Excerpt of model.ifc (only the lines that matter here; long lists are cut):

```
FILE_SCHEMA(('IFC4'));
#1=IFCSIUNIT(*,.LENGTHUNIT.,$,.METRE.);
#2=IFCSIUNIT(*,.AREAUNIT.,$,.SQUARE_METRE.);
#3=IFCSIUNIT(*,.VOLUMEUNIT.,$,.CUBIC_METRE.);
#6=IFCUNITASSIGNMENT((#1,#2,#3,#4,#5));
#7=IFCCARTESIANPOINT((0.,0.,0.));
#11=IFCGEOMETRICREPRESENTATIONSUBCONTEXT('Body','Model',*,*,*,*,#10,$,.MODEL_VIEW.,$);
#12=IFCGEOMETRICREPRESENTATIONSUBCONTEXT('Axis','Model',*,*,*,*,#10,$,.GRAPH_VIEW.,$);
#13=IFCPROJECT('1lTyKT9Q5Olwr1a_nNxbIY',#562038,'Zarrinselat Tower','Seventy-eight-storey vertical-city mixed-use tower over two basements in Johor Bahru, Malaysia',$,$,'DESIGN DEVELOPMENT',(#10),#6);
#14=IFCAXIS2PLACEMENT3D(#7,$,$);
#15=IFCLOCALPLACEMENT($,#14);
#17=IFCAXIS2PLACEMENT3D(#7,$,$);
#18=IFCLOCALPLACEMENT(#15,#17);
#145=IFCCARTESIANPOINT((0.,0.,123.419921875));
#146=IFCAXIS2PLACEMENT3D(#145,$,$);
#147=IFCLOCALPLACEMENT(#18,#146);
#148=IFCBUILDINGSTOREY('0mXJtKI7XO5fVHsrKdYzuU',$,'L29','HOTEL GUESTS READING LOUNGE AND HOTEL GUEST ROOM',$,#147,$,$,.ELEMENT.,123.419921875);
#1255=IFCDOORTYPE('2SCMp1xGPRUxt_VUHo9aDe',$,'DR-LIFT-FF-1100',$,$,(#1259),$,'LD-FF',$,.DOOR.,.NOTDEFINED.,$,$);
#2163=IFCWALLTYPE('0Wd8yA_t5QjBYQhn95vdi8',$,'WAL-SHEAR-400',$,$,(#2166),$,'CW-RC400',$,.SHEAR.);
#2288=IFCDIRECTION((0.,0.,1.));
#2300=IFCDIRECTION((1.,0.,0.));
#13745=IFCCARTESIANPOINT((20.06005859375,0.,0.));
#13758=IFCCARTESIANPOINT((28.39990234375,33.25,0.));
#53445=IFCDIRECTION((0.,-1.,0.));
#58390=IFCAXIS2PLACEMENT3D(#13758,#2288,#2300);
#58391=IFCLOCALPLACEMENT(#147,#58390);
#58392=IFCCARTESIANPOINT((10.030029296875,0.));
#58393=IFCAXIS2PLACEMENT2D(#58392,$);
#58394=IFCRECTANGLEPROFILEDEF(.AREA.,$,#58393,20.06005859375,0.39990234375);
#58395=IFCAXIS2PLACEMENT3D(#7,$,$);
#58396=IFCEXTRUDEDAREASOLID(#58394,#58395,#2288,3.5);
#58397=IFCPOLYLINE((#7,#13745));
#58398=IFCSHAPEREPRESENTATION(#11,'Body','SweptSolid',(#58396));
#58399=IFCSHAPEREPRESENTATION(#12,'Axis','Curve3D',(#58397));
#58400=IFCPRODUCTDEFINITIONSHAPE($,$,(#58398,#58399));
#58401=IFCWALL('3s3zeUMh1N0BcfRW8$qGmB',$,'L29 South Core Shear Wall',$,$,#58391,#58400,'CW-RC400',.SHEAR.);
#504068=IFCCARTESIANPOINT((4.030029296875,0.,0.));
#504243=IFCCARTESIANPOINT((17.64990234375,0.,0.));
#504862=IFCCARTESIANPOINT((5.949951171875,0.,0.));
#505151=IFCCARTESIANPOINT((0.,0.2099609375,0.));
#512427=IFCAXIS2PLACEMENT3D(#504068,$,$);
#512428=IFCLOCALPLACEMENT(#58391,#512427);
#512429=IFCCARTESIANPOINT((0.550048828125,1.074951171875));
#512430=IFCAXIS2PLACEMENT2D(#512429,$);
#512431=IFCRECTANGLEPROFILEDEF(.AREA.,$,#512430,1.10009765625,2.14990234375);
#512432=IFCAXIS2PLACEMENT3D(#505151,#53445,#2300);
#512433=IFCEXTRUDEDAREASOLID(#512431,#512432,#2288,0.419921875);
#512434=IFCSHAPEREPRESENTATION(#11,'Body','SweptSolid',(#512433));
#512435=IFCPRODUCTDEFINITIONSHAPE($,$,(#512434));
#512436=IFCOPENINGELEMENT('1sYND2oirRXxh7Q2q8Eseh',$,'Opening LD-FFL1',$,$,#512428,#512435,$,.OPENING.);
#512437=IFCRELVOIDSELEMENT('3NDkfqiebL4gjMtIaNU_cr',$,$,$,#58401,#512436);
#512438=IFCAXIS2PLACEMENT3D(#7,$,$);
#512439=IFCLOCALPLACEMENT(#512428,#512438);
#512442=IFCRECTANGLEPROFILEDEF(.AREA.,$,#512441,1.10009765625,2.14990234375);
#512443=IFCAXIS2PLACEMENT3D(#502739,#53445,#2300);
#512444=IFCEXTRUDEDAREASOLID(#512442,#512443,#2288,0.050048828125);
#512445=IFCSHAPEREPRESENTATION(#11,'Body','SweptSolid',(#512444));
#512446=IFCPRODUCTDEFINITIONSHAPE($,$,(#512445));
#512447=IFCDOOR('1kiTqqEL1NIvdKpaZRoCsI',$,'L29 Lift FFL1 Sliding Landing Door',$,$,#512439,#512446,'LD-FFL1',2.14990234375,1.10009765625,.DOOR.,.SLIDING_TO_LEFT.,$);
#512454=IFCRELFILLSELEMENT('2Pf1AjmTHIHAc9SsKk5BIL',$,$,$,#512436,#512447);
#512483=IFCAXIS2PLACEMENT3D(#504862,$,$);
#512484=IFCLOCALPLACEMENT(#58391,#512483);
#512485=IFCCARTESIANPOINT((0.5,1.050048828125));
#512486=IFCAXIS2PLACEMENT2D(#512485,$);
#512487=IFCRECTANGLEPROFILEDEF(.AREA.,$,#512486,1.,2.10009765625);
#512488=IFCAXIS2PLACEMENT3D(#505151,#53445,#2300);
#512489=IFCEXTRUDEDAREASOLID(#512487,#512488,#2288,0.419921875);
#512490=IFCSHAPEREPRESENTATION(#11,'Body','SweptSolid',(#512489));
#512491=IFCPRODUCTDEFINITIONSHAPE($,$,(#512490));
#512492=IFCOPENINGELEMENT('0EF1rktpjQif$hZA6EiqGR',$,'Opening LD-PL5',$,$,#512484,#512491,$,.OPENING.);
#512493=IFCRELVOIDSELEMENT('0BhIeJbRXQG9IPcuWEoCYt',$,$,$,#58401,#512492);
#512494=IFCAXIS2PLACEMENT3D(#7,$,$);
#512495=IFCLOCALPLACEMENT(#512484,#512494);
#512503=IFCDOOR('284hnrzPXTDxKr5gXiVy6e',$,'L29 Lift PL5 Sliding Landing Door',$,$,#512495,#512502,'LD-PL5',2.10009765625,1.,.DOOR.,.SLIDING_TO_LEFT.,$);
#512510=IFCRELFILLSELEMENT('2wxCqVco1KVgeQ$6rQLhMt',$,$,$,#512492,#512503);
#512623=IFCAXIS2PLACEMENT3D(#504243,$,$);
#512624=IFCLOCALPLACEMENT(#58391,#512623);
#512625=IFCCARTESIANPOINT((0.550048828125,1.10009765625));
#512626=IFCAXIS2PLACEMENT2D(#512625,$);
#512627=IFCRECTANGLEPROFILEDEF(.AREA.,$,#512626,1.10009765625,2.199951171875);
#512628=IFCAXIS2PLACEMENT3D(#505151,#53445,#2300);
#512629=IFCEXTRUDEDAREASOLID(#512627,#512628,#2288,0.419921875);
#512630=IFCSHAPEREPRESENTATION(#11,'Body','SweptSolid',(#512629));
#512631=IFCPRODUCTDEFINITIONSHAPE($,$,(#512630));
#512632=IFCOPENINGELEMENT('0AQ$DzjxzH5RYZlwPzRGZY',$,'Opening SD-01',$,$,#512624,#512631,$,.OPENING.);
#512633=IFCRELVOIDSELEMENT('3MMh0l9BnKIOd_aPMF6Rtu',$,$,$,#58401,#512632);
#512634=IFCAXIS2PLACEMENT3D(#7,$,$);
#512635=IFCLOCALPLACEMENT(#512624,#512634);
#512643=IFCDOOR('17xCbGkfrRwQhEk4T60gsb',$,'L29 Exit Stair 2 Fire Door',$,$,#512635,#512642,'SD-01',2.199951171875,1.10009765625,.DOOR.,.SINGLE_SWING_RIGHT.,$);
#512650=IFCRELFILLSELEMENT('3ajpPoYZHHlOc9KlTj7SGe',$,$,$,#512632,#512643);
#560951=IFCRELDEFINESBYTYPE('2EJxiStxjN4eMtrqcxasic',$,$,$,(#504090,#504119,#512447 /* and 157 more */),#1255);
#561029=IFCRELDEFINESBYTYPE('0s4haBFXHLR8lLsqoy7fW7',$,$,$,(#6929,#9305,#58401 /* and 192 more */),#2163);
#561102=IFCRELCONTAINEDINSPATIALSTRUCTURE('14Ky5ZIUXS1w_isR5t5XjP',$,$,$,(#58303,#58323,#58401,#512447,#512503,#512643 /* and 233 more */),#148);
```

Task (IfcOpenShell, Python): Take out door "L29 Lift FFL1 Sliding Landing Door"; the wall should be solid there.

```python
import ifcopenshell
import ifcopenshell.api.feature
import ifcopenshell.api.root
import ifcopenshell.geom
import ifcopenshell.util.shape

model = ifcopenshell.open("model.ifc")
settings = ifcopenshell.geom.settings()


def volume(element):
    """Net volume in cubic metres, openings subtracted."""
    shape = ifcopenshell.geom.create_shape(settings, element)
    return ifcopenshell.util.shape.get_volume(shape.geometry)


door = model.by_guid("1kiTqqEL1NIvdKpaZRoCsI")
opening = door.FillsVoids[0].RelatingOpeningElement
wall = opening.VoidsElements[0].RelatingBuildingElement
before = volume(wall)

ifcopenshell.api.root.remove_product(model, product=door)
ifcopenshell.api.feature.remove_feature(model, feature=opening)

after = volume(wall)

print(f"wall volume {before:.3f} -> {after:.3f} m3")

model.write("model_edited.ifc")
```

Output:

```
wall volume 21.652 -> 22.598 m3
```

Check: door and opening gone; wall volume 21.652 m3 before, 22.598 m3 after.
